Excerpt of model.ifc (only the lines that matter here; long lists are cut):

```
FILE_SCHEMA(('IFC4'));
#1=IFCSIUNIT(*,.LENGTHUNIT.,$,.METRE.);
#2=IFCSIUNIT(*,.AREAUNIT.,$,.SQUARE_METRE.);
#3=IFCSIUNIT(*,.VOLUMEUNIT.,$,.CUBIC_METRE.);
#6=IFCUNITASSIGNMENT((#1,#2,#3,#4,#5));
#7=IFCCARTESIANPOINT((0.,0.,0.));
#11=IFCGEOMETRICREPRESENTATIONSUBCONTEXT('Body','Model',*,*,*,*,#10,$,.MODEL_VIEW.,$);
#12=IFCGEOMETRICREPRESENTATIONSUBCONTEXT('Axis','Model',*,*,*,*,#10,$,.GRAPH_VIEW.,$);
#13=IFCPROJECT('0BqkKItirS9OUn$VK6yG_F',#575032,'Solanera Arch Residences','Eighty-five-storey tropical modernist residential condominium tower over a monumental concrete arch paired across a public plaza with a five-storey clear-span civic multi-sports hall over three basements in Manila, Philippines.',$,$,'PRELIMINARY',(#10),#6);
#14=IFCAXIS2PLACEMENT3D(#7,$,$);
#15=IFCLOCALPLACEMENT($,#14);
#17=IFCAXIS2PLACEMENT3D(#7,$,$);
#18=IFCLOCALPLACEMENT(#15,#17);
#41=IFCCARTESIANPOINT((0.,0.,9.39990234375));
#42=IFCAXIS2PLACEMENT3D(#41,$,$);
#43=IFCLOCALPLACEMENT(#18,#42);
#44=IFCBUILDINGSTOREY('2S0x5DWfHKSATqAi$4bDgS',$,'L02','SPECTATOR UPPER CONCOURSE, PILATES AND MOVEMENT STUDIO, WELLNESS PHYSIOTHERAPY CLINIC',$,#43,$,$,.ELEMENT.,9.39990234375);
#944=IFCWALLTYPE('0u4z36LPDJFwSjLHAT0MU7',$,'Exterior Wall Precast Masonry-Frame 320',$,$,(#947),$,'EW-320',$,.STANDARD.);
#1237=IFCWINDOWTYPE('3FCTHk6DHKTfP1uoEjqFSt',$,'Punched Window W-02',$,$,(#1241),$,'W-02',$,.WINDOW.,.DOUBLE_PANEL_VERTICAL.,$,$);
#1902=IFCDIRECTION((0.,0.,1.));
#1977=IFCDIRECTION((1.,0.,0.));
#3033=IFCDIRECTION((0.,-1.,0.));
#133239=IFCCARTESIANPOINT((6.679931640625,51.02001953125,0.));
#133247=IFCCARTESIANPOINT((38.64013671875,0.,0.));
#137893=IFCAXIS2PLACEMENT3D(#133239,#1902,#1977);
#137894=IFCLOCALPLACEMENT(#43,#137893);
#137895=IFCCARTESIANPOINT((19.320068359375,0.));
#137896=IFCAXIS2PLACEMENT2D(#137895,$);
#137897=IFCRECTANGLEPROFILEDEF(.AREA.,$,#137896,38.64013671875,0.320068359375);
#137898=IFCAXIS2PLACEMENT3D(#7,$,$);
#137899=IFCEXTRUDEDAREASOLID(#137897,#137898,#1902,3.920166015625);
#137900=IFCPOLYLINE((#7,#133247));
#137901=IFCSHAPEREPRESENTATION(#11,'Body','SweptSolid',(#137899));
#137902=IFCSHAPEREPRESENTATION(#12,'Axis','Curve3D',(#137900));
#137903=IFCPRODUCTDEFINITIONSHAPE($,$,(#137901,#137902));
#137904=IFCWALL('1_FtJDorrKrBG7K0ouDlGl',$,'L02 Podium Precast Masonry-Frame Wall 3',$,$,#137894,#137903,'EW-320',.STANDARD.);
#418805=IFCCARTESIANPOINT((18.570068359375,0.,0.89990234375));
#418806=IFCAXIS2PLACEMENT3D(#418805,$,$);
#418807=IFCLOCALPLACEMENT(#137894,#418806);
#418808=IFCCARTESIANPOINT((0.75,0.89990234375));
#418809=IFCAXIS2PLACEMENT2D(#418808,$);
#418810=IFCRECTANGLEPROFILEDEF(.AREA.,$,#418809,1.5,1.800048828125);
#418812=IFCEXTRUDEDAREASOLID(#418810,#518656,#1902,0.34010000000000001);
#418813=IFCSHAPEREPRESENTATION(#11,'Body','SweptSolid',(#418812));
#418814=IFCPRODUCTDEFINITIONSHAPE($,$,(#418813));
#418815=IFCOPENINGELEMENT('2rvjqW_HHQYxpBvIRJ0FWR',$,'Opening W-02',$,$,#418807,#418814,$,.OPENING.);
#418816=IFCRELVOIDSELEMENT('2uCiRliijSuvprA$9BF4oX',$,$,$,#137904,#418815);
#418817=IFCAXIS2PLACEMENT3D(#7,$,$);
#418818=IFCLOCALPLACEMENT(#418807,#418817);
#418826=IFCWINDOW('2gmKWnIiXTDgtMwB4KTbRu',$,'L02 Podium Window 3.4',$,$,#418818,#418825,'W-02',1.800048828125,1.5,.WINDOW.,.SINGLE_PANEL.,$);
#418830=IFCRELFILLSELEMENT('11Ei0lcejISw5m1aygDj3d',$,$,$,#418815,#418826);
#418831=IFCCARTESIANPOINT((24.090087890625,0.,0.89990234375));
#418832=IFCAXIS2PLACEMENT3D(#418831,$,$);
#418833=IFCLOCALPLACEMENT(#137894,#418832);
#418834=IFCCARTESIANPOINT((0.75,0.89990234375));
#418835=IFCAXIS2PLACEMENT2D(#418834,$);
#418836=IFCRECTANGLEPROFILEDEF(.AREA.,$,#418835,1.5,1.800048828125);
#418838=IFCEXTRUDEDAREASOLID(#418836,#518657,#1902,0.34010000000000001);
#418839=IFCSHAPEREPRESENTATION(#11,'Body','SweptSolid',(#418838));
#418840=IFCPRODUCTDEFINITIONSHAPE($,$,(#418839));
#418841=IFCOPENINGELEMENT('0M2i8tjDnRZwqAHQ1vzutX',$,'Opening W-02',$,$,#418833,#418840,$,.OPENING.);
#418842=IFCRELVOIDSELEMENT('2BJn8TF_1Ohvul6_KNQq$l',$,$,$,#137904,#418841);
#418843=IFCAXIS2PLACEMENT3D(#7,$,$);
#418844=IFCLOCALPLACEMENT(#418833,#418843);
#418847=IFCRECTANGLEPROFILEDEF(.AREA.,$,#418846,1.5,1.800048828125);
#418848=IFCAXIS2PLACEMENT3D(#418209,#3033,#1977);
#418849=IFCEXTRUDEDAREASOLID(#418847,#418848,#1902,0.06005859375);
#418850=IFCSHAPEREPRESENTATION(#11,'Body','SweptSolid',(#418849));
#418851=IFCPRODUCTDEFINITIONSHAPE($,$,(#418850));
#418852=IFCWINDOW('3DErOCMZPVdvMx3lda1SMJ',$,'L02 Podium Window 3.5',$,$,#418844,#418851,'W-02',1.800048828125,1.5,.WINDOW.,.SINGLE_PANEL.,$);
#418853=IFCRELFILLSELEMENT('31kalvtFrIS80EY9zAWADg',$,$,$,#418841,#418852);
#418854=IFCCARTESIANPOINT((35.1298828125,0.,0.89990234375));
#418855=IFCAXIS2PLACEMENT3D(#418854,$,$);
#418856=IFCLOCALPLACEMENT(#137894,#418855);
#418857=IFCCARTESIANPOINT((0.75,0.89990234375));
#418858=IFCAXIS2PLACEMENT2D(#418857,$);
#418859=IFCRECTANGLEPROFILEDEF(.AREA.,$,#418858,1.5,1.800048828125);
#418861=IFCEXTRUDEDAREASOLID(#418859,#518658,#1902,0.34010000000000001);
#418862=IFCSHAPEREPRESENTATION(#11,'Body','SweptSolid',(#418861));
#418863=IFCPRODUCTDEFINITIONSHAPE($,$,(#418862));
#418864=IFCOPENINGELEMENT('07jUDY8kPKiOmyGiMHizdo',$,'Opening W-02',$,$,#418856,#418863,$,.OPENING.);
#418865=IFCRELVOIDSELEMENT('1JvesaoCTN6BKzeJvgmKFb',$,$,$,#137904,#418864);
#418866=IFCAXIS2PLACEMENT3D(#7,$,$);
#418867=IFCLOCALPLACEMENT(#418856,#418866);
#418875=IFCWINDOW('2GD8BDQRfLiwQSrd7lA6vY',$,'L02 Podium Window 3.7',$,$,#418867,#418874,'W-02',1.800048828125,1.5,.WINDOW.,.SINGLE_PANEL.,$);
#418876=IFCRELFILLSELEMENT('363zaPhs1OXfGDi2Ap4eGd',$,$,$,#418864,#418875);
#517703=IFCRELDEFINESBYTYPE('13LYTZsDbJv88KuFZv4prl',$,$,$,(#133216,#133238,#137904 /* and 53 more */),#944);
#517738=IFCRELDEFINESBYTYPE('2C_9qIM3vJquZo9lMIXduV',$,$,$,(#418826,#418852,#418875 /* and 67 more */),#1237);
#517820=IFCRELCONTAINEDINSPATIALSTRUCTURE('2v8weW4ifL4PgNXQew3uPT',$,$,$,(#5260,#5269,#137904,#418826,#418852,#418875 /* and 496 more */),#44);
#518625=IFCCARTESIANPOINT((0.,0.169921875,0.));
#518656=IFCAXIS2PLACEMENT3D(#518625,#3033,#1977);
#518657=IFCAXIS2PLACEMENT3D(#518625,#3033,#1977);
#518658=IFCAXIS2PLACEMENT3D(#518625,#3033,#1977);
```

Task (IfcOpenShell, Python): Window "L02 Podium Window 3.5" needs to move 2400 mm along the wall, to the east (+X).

```python
import ifcopenshell
import ifcopenshell.api.geometry
import ifcopenshell.util.placement

model = ifcopenshell.open("model.ifc")

window = model.by_guid("3DErOCMZPVdvMx3lda1SMJ")
opening = window.FillsVoids[0].RelatingOpeningElement
wall = opening.VoidsElements[0].RelatingBuildingElement

wall_matrix = ifcopenshell.util.placement.get_local_placement(wall.ObjectPlacement)
shift = wall_matrix[:3, 0] * 2.4
before = ifcopenshell.util.placement.get_local_placement(window.ObjectPlacement)[:3, 3].copy()

# The window is placed relative to its opening, so it follows when the opening moves.
matrix = ifcopenshell.util.placement.get_local_placement(opening.ObjectPlacement)
matrix[:3, 3] += shift
ifcopenshell.api.geometry.edit_object_placement(
    model, product=opening, matrix=matrix, is_si=False, should_transform_children=True
)

after = ifcopenshell.util.placement.get_local_placement(window.ObjectPlacement)[:3, 3]
print("window moved by", (after - before).round(3) + 0.0)

model.write("model_updated.ifc")
```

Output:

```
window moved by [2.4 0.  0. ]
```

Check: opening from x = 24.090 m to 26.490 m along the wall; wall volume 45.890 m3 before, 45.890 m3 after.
